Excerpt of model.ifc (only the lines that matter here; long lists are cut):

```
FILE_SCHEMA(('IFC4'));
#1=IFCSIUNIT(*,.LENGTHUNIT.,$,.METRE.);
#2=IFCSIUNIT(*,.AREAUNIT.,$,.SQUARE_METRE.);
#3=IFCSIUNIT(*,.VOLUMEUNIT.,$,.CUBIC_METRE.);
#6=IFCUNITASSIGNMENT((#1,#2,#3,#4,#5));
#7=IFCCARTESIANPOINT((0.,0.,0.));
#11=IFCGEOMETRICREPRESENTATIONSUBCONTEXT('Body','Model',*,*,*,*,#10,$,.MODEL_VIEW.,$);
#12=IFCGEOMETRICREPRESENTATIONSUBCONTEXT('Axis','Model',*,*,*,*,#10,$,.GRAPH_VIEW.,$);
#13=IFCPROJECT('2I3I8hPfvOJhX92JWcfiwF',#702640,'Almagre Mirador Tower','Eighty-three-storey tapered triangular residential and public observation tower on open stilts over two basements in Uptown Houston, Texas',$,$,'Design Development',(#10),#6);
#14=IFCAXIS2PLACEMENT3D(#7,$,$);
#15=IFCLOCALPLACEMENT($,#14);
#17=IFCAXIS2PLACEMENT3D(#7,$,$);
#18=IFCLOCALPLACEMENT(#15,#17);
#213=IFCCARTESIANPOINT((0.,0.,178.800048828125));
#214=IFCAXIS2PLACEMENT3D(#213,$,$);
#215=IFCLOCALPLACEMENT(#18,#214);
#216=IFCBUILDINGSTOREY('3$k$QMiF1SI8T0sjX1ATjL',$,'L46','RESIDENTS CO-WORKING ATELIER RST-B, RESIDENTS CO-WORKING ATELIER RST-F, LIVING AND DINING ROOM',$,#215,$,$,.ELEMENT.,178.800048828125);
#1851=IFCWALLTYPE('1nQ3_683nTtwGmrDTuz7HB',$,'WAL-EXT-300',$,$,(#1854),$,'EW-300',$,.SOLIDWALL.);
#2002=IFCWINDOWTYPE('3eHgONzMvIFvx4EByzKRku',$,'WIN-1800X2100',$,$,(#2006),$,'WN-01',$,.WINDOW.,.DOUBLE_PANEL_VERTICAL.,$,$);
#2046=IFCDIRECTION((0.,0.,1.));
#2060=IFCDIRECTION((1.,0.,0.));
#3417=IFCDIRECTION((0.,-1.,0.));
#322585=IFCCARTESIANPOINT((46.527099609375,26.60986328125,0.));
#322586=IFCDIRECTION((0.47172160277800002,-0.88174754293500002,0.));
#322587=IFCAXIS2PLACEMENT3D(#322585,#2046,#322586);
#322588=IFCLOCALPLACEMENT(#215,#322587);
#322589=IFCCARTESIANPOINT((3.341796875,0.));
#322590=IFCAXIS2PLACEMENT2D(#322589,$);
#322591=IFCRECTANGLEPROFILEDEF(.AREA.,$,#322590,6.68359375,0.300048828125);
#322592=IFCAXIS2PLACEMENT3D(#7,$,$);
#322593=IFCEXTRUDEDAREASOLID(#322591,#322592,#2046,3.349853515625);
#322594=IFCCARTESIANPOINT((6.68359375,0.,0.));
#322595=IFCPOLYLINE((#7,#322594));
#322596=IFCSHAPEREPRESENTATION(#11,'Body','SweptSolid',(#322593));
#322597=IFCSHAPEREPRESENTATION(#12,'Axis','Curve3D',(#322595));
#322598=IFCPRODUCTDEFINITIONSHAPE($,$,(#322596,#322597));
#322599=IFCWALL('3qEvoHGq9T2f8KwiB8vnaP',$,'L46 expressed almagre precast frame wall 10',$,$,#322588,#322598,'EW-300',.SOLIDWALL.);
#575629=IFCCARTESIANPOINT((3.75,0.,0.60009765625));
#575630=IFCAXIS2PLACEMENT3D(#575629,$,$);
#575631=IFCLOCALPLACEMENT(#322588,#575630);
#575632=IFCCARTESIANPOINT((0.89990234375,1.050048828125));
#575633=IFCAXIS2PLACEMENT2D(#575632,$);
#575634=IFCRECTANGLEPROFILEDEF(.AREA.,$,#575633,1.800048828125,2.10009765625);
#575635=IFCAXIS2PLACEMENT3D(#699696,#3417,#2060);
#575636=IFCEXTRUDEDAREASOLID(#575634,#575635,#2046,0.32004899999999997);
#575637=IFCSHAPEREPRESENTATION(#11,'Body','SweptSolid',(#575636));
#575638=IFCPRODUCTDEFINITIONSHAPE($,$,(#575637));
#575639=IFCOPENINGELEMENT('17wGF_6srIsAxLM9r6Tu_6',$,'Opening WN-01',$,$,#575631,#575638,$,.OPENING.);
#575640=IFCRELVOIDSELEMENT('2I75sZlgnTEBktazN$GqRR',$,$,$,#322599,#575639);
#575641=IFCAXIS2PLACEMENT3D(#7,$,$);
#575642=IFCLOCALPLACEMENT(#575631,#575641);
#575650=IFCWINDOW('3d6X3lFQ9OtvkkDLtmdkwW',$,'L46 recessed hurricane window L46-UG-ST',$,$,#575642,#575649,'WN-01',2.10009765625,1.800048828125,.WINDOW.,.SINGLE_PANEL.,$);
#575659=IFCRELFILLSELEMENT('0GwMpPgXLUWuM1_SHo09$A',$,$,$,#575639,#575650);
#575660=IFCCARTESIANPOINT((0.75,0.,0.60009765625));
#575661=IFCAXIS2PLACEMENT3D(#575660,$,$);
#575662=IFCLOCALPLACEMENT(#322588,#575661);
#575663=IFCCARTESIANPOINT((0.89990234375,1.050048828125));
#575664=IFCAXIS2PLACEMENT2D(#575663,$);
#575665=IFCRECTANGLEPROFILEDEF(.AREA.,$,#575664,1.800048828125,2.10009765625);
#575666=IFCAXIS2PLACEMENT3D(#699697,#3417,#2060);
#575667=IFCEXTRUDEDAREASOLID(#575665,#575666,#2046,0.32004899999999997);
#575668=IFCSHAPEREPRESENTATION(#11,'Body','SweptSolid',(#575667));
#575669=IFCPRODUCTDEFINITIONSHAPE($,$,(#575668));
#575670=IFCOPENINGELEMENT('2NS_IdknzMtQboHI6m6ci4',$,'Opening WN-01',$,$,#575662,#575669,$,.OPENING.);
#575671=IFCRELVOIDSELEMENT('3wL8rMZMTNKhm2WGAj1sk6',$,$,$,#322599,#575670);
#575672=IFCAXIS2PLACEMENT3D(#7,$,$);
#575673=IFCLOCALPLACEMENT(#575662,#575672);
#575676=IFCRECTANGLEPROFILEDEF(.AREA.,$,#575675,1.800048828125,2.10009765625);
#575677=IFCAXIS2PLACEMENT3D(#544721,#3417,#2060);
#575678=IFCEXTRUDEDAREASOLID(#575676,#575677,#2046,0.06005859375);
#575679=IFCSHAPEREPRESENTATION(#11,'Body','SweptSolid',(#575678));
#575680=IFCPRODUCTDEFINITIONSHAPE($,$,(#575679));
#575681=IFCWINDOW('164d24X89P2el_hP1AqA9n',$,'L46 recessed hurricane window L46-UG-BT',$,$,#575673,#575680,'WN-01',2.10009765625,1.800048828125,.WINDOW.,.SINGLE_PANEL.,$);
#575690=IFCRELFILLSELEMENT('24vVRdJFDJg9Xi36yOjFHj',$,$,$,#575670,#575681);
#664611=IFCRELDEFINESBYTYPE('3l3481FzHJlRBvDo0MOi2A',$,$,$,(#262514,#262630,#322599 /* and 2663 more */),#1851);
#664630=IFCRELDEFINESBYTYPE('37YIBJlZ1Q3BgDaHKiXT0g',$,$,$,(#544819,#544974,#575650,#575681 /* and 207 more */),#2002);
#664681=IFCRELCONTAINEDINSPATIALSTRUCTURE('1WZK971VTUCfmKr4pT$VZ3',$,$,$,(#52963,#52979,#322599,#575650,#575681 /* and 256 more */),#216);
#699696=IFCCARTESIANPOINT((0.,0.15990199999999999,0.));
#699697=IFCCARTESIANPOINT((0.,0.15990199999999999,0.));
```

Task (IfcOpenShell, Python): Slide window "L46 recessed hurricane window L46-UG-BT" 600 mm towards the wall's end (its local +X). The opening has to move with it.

```python
import ifcopenshell
import ifcopenshell.api.geometry
import ifcopenshell.util.placement
import ifcopenshell.util.unit

model = ifcopenshell.open("model.ifc")
unit_scale = ifcopenshell.util.unit.calculate_unit_scale(model)

window = model.by_guid("164d24X89P2el_hP1AqA9n")
opening = window.FillsVoids[0].RelatingOpeningElement
wall = opening.VoidsElements[0].RelatingBuildingElement

wall_matrix = ifcopenshell.util.placement.get_local_placement(wall.ObjectPlacement)
shift = wall_matrix[:3, 0] * 0.6 / unit_scale
before = ifcopenshell.util.placement.get_local_placement(window.ObjectPlacement)[:3, 3].copy()

# The window is placed relative to its opening, so it follows when the opening moves.
matrix = ifcopenshell.util.placement.get_local_placement(opening.ObjectPlacement)
matrix[:3, 3] += shift
ifcopenshell.api.geometry.edit_object_placement(
    model, product=opening, matrix=matrix, is_si=False, should_transform_children=True
)

after = ifcopenshell.util.placement.get_local_placement(window.ObjectPlacement)[:3, 3]
print("window moved by", (after - before).round(3) + 0.0)

model.write("model_v2.ifc")
```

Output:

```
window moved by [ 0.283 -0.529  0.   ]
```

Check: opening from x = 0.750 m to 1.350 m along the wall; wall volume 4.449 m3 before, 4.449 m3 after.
